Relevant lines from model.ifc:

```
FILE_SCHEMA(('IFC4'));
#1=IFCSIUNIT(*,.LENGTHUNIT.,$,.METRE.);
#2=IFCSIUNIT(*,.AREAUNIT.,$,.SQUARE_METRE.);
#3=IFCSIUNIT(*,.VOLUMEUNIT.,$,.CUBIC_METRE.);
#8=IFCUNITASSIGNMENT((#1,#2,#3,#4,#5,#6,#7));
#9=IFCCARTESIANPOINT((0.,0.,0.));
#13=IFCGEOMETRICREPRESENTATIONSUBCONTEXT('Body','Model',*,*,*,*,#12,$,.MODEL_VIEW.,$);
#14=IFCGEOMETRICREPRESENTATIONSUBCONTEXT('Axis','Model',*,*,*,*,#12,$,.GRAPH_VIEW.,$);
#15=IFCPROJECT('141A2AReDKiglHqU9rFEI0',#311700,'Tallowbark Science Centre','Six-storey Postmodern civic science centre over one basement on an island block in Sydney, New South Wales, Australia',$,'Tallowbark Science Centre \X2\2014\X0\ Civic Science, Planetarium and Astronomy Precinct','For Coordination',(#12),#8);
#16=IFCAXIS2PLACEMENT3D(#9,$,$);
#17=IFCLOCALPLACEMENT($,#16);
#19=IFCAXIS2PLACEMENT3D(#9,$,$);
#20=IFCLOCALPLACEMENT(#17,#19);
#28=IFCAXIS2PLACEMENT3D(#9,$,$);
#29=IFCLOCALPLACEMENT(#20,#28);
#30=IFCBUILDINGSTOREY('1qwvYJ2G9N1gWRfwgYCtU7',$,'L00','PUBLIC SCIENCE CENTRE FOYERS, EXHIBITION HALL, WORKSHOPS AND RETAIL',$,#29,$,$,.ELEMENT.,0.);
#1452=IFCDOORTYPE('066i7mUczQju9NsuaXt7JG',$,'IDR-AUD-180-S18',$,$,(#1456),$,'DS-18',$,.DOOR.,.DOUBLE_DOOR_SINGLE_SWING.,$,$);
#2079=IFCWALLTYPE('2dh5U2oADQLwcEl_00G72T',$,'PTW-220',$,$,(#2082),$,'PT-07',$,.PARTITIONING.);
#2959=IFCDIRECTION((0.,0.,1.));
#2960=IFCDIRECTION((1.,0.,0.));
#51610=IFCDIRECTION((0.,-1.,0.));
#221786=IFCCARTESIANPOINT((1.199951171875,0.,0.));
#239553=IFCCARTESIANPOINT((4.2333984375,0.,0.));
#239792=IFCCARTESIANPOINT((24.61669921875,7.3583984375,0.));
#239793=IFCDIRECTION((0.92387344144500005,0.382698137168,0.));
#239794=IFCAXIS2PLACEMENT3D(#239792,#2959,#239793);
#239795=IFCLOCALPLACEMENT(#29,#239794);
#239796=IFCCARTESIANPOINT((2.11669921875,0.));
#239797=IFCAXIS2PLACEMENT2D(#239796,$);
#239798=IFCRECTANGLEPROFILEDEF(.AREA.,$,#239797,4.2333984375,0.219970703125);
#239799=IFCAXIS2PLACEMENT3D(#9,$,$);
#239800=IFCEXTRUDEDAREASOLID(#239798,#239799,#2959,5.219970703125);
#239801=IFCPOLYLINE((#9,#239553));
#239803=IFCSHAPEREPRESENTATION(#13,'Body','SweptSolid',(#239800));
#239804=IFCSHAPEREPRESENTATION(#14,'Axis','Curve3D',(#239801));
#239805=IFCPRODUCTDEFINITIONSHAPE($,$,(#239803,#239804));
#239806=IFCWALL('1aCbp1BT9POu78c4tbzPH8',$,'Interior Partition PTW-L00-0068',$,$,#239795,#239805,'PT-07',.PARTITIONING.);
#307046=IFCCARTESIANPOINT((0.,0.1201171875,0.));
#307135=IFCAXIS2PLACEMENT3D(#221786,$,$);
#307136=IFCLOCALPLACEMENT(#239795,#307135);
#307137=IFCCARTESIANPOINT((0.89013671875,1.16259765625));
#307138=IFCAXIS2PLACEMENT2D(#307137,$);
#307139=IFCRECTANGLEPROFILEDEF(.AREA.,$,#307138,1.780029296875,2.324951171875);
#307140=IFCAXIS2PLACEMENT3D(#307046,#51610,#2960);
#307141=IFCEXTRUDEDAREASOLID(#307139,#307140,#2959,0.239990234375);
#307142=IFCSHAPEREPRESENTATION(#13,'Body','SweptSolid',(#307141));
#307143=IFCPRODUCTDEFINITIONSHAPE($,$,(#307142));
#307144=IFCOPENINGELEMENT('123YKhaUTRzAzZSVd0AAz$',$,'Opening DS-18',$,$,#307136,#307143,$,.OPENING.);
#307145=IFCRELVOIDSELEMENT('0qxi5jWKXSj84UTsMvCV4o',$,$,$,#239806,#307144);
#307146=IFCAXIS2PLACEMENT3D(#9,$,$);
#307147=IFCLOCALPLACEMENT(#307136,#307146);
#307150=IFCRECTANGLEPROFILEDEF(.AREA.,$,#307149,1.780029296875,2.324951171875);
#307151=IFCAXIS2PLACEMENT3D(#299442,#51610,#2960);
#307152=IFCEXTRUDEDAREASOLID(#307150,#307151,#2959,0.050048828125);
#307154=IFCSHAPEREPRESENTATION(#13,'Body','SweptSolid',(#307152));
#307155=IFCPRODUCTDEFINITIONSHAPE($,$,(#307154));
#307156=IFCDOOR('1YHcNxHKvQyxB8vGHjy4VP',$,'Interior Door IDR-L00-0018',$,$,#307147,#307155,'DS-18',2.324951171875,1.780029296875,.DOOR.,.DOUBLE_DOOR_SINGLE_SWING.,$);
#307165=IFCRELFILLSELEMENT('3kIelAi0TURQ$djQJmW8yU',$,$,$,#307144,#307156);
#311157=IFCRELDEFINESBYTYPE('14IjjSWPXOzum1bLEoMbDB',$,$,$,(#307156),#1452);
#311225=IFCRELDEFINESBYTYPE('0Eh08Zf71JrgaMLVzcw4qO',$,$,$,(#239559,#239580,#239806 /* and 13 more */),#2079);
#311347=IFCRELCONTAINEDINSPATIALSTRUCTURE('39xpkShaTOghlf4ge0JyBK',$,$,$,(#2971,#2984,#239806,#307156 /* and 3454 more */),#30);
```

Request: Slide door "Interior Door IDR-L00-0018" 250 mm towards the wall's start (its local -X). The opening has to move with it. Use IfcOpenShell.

```python
import ifcopenshell
import ifcopenshell.api.geometry
import ifcopenshell.util.placement

model = ifcopenshell.open("model.ifc")

door = model.by_id(307156)
opening = door.FillsVoids[0].RelatingOpeningElement
wall = opening.VoidsElements[0].RelatingBuildingElement

wall_matrix = ifcopenshell.util.placement.get_local_placement(wall.ObjectPlacement)
shift = wall_matrix[:3, 0] * -0.25
before = ifcopenshell.util.placement.get_local_placement(door.ObjectPlacement)[:3, 3].copy()

# The door is placed relative to its opening, so it follows when the opening moves.
matrix = ifcopenshell.util.placement.get_local_placement(opening.ObjectPlacement)
matrix[:3, 3] += shift
ifcopenshell.api.geometry.edit_object_placement(
    model, product=opening, matrix=matrix, is_si=False, should_transform_children=True
)

after = ifcopenshell.util.placement.get_local_placement(door.ObjectPlacement)[:3, 3]
print("door moved by", (after - before).round(3) + 0.0)

model.write("model_v2.ifc")
```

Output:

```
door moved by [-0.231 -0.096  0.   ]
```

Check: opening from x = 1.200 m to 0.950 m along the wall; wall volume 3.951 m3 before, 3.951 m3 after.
